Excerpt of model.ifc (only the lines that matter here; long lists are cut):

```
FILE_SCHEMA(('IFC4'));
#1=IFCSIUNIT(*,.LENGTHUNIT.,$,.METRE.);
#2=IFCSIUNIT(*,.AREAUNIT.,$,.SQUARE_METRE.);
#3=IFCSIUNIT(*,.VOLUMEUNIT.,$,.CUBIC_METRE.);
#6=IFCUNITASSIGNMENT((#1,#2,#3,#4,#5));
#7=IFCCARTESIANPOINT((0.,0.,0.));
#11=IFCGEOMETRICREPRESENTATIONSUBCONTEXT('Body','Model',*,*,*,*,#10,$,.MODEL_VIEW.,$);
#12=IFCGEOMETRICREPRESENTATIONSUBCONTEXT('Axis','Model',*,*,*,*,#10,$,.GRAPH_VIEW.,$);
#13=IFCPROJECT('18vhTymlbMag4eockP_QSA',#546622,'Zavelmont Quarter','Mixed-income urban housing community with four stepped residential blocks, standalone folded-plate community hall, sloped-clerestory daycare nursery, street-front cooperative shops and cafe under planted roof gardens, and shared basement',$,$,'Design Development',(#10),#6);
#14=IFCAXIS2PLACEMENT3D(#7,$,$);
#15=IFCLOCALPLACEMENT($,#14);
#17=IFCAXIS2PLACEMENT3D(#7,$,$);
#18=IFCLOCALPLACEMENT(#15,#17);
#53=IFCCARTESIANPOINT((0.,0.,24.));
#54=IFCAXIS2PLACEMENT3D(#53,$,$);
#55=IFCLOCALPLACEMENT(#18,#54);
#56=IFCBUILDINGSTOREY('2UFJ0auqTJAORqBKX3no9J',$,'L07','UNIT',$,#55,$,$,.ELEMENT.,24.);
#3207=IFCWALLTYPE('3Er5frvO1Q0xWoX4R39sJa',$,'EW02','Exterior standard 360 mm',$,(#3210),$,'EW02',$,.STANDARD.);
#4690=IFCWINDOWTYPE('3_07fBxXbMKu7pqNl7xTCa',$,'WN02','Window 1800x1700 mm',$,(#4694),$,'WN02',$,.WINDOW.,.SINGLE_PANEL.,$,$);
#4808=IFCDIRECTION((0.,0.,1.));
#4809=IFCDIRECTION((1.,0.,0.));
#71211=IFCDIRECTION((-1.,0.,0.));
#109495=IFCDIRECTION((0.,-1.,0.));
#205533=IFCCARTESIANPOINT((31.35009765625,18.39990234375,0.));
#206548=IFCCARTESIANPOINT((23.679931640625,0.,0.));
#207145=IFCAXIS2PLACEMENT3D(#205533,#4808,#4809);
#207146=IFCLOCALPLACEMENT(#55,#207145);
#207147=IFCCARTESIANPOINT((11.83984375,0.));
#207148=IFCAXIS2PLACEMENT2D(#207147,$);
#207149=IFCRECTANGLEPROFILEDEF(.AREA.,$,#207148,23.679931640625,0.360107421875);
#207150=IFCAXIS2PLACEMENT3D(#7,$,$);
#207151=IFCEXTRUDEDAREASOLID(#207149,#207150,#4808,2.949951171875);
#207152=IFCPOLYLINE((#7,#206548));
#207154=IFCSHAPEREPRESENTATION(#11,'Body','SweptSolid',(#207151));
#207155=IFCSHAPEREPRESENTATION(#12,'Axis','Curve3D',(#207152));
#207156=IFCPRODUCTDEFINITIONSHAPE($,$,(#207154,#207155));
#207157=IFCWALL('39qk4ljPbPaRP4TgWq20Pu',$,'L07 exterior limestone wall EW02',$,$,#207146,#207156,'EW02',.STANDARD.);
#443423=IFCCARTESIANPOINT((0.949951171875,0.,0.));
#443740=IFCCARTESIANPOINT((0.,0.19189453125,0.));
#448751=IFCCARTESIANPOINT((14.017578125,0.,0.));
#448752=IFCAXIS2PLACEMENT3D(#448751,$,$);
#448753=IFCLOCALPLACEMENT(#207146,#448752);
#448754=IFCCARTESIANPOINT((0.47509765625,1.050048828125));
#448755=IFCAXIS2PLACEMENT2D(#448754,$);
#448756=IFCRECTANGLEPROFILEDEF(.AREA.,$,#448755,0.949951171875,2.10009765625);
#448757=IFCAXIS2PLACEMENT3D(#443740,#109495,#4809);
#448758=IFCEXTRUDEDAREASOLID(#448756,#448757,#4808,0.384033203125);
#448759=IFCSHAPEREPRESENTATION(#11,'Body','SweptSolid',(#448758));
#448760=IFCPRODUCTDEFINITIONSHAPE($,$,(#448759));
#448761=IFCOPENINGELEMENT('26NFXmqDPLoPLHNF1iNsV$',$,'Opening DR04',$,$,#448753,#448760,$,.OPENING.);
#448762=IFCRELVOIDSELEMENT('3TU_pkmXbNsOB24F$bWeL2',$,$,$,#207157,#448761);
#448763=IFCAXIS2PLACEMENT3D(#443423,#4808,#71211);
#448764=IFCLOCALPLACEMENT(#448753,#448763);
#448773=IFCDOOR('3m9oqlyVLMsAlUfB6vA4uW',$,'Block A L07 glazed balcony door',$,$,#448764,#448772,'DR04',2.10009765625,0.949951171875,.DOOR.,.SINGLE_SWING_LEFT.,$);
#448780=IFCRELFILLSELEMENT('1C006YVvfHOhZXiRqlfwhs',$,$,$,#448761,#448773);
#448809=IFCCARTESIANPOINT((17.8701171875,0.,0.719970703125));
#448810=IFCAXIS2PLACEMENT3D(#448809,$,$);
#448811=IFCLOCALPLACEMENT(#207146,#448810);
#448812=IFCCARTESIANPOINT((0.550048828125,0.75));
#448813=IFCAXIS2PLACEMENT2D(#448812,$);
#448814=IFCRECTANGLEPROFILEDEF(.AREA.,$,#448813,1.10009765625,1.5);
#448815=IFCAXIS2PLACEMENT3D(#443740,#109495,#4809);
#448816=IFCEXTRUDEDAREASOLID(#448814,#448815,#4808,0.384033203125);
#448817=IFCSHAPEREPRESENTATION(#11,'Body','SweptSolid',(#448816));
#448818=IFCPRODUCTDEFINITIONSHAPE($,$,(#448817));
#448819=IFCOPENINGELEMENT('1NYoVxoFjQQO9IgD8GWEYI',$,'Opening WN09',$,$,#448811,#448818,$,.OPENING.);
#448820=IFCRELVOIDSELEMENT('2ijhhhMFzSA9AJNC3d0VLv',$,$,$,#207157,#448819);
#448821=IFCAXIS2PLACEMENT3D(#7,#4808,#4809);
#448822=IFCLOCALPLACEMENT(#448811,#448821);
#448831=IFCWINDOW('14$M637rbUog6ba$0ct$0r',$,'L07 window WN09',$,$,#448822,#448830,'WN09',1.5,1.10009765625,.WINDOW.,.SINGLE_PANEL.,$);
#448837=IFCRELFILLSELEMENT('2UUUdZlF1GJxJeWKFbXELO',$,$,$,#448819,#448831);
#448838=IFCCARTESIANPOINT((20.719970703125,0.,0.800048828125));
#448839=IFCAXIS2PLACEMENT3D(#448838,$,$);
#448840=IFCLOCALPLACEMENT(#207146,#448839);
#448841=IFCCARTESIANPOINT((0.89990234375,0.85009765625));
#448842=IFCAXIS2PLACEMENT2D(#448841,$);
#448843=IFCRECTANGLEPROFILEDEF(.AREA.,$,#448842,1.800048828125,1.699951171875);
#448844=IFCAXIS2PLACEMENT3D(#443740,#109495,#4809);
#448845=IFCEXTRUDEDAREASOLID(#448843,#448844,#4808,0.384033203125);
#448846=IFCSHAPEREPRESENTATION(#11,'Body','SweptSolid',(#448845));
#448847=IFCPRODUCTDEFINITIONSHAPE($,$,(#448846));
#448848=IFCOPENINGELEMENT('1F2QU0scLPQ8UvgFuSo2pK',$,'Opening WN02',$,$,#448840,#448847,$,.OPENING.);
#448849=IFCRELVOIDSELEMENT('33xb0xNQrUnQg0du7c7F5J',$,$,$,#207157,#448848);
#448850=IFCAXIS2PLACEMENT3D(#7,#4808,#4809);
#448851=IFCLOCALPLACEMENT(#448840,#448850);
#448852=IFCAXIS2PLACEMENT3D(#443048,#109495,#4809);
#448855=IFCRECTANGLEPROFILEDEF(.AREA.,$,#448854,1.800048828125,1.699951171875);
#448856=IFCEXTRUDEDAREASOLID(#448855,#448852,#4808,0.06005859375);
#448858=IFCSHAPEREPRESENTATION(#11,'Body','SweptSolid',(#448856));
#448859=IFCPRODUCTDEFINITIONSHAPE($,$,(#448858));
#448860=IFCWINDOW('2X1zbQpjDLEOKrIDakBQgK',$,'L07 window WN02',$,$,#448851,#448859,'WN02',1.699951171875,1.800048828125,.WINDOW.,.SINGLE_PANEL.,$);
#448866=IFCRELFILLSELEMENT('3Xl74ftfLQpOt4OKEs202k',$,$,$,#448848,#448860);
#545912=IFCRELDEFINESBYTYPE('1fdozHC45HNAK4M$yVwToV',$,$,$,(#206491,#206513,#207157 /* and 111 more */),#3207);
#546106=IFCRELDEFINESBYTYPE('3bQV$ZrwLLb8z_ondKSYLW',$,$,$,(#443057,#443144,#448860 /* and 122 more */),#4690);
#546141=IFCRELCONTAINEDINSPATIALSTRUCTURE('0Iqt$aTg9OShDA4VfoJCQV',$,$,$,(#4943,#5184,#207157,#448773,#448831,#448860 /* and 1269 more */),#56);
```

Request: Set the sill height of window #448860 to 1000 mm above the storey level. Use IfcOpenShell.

```python
import numpy as np
import ifcopenshell
import ifcopenshell.api.geometry
import ifcopenshell.geom
import ifcopenshell.util.element
import ifcopenshell.util.placement
import ifcopenshell.util.shape
import ifcopenshell.util.unit

model = ifcopenshell.open("model.ifc")
unit_scale = ifcopenshell.util.unit.calculate_unit_scale(model)

window = model.by_id(448860)
opening = window.FillsVoids[0].RelatingOpeningElement
storey = ifcopenshell.util.element.get_container(window, ifc_class="IfcBuildingStorey")
level = ifcopenshell.util.placement.get_local_placement(storey.ObjectPlacement)[2, 3]

# The opening's origin need not be at the sill, so measure its lowest point.
shape = ifcopenshell.geom.create_shape(ifcopenshell.geom.settings(), opening)
bottom = ifcopenshell.util.shape.get_shape_bottom_elevation(shape, shape.geometry) / unit_scale
dz = level + 1.0 - bottom

shift = np.array([0.0, 0.0, dz])
# The window is placed relative to its opening, so it follows when the opening moves.
matrix = ifcopenshell.util.placement.get_local_placement(opening.ObjectPlacement)
matrix[:3, 3] += shift
ifcopenshell.api.geometry.edit_object_placement(
    model, product=opening, matrix=matrix, is_si=False, should_transform_children=True
)

print(f"moved by {dz * unit_scale:+.3f} m")

model.write("model_updated.ifc")
```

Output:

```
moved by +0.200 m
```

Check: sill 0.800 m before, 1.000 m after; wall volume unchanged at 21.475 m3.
